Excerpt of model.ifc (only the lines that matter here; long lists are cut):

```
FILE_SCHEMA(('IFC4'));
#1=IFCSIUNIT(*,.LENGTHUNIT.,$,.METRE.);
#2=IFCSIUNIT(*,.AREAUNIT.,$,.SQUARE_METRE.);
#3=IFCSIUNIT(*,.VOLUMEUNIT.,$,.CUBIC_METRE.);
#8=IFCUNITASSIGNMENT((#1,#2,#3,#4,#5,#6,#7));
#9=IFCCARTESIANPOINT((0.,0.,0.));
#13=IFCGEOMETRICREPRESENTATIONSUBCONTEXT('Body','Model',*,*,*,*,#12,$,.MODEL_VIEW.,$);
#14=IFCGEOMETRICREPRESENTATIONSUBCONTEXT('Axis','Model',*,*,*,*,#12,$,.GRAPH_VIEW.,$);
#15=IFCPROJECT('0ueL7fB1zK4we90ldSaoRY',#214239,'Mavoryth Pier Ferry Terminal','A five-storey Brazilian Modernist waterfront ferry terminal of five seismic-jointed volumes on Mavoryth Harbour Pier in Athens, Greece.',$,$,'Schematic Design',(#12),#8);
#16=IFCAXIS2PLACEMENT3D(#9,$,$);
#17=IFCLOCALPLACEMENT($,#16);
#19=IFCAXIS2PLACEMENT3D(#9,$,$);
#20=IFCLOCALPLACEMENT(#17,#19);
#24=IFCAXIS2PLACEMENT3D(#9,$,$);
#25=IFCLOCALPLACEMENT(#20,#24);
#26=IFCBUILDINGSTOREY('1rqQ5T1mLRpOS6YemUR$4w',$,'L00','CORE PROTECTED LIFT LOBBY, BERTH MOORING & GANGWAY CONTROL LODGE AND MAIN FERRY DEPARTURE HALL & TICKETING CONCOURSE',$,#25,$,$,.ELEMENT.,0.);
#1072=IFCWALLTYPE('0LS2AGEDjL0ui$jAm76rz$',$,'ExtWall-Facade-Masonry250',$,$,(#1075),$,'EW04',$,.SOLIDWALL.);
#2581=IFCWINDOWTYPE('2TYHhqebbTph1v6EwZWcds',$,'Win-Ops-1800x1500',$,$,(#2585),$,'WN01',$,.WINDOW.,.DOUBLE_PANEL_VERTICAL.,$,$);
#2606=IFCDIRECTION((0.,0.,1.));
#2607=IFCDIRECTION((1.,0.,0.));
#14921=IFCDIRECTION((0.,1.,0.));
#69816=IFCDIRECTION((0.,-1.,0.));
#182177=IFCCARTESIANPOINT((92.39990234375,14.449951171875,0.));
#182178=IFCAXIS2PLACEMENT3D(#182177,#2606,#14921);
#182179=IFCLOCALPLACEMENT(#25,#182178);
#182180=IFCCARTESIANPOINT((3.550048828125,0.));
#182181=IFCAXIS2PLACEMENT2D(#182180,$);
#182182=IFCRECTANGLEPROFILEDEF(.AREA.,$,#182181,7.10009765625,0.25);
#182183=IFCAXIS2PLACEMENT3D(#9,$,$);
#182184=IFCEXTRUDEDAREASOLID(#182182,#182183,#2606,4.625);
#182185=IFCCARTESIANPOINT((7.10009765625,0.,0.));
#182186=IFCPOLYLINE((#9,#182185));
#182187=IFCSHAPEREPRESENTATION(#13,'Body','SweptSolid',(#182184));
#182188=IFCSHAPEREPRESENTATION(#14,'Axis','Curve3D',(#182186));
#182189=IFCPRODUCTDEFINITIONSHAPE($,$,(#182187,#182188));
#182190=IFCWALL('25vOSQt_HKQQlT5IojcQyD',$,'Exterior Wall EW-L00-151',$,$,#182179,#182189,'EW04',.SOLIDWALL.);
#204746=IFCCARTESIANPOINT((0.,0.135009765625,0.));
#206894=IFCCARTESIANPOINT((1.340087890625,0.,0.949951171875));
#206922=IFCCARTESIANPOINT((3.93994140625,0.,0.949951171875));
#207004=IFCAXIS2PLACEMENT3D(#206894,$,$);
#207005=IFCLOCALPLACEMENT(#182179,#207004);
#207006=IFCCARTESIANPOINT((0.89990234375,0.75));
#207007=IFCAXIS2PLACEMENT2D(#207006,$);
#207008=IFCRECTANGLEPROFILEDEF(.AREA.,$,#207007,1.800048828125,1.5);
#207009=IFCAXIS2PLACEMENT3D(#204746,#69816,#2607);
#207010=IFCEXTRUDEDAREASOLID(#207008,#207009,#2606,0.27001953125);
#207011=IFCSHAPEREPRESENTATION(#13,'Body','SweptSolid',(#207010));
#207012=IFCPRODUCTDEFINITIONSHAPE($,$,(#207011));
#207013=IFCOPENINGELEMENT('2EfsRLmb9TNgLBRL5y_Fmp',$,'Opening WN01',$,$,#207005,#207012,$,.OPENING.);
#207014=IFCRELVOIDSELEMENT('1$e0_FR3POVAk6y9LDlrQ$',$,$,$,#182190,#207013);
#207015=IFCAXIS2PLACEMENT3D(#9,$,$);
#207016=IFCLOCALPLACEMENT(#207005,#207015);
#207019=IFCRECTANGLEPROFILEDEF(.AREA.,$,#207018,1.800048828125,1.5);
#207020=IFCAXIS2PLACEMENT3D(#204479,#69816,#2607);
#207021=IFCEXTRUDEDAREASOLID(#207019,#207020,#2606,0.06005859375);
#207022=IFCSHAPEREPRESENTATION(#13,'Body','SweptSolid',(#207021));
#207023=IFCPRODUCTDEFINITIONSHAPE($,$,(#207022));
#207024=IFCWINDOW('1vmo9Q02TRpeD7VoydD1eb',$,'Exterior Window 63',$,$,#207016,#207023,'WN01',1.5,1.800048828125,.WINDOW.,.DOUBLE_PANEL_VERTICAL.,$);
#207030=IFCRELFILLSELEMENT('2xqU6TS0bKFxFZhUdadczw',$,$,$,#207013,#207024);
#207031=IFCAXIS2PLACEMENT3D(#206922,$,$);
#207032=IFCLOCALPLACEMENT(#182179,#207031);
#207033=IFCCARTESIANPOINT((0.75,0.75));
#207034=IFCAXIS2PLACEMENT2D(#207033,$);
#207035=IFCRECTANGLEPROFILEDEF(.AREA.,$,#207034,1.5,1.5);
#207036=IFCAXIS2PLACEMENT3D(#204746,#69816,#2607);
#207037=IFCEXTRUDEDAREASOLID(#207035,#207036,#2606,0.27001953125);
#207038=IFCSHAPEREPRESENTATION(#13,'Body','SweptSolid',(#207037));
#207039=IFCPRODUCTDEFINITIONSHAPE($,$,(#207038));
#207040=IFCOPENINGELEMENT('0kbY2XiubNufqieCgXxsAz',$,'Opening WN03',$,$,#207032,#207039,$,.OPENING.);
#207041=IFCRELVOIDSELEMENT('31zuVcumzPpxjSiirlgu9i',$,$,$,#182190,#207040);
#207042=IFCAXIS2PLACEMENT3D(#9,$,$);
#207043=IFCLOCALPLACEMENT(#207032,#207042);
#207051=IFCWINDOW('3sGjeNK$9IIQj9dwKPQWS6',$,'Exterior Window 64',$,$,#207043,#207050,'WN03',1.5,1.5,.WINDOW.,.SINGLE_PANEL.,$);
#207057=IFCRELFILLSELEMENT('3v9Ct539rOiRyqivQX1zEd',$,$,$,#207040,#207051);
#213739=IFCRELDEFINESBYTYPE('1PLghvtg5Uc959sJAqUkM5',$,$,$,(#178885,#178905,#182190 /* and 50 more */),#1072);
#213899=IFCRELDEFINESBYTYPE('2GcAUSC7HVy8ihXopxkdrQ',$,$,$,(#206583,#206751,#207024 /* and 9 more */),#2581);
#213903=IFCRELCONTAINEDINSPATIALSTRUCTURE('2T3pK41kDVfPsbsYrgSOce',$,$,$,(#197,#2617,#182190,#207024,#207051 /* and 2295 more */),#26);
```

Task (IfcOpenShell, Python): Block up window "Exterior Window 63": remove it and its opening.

```python
import ifcopenshell
import ifcopenshell.api.feature
import ifcopenshell.api.root
import ifcopenshell.geom
import ifcopenshell.util.shape

model = ifcopenshell.open("model.ifc")
settings = ifcopenshell.geom.settings()


def volume(element):
    """Net volume in cubic metres, openings subtracted."""
    shape = ifcopenshell.geom.create_shape(settings, element)
    return ifcopenshell.util.shape.get_volume(shape.geometry)


window = model.by_guid("1vmo9Q02TRpeD7VoydD1eb")
opening = window.FillsVoids[0].RelatingOpeningElement
wall = opening.VoidsElements[0].RelatingBuildingElement
before = volume(wall)

ifcopenshell.api.root.remove_product(model, product=window)
ifcopenshell.api.feature.remove_feature(model, feature=opening)

after = volume(wall)

print(f"wall volume {before:.3f} -> {after:.3f} m3")

model.write("model_rev.ifc")
```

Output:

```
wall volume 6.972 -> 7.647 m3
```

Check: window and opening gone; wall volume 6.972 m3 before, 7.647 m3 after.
